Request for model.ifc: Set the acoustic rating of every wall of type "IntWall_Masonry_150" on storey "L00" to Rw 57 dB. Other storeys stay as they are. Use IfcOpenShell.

First a look at what the model holds.

```python
import ifcopenshell
import ifcopenshell.util.element

model = ifcopenshell.open("model.ifc")
print(model.schema)
storey = next(s for s in model.by_type("IfcBuildingStorey") if s.Name == "L00")
walls = [e for e in ifcopenshell.util.element.get_decomposition(storey) if e.is_a("IfcWall")]
seen = {}
for e in walls:
    element_type = ifcopenshell.util.element.get_type(e)
    key = (element_type.Name if element_type != e and element_type else None, ifcopenshell.util.element.get_pset(e, "Pset_WallCommon", "AcousticRating"))
    seen[key] = seen.get(key, 0) + 1
for (name, value), count in sorted(seen.items(), key=str):
    print(count, "x", name, "|", value)
```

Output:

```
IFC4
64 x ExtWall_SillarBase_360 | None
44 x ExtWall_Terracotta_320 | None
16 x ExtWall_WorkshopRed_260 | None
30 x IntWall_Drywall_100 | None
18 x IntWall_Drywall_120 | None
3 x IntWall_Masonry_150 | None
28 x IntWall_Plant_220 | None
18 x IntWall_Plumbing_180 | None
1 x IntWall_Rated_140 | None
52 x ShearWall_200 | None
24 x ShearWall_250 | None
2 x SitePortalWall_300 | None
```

```python
import ifcopenshell
import ifcopenshell.api.pset
import ifcopenshell.util.element

model = ifcopenshell.open("model.ifc")

storey = next(s for s in model.by_type("IfcBuildingStorey") if s.Name == "L00")
walls = [e for e in ifcopenshell.util.element.get_decomposition(storey) if e.is_a("IfcWall")]

count = 0
for e in walls:
    element_type = ifcopenshell.util.element.get_type(e)
    if element_type in (None, e) or element_type.Name != "IntWall_Masonry_150":
        continue
    # add_pset returns the element's existing set when there is one.
    pset = ifcopenshell.api.pset.add_pset(model, product=e, name="Pset_WallCommon")
    ifcopenshell.api.pset.edit_pset(model, pset=pset, properties={"AcousticRating": "Rw 57 dB"})
    count += 1

print(count, "walls updated")

model.write("model_v2.ifc")
```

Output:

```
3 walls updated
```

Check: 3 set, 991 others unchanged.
